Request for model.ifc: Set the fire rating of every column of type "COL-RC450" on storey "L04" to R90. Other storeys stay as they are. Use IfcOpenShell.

First a look at what the model holds.

```python
import ifcopenshell
import ifcopenshell.util.element

model = ifcopenshell.open("model.ifc")
print(model.schema)
storey = next(s for s in model.by_type("IfcBuildingStorey") if s.Name == "L04")
columns = [e for e in ifcopenshell.util.element.get_decomposition(storey) if e.is_a("IfcColumn")]
seen = {}
for e in columns:
    element_type = ifcopenshell.util.element.get_type(e)
    key = (element_type.Name if element_type != e and element_type else None, ifcopenshell.util.element.get_pset(e, "Pset_ColumnCommon", "FireRating"))
    seen[key] = seen.get(key, 0) + 1
for (name, value), count in sorted(seen.items(), key=str):
    print(count, "x", name, "|", value)
```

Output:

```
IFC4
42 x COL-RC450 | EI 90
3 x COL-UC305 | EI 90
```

```python
import ifcopenshell
import ifcopenshell.api.pset
import ifcopenshell.util.element

model = ifcopenshell.open("model.ifc")

storey = next(s for s in model.by_type("IfcBuildingStorey") if s.Name == "L04")
columns = [e for e in ifcopenshell.util.element.get_decomposition(storey) if e.is_a("IfcColumn")]

count = 0
for e in columns:
    element_type = ifcopenshell.util.element.get_type(e)
    if element_type in (None, e) or element_type.Name != "COL-RC450":
        continue
    # add_pset returns the element's existing set when there is one.
    pset = ifcopenshell.api.pset.add_pset(model, product=e, name="Pset_ColumnCommon")
    ifcopenshell.api.pset.edit_pset(model, pset=pset, properties={"FireRating": "R90"})
    count += 1

print(count, "columns updated")

model.write("model_edited.ifc")
```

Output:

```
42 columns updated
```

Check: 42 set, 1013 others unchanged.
